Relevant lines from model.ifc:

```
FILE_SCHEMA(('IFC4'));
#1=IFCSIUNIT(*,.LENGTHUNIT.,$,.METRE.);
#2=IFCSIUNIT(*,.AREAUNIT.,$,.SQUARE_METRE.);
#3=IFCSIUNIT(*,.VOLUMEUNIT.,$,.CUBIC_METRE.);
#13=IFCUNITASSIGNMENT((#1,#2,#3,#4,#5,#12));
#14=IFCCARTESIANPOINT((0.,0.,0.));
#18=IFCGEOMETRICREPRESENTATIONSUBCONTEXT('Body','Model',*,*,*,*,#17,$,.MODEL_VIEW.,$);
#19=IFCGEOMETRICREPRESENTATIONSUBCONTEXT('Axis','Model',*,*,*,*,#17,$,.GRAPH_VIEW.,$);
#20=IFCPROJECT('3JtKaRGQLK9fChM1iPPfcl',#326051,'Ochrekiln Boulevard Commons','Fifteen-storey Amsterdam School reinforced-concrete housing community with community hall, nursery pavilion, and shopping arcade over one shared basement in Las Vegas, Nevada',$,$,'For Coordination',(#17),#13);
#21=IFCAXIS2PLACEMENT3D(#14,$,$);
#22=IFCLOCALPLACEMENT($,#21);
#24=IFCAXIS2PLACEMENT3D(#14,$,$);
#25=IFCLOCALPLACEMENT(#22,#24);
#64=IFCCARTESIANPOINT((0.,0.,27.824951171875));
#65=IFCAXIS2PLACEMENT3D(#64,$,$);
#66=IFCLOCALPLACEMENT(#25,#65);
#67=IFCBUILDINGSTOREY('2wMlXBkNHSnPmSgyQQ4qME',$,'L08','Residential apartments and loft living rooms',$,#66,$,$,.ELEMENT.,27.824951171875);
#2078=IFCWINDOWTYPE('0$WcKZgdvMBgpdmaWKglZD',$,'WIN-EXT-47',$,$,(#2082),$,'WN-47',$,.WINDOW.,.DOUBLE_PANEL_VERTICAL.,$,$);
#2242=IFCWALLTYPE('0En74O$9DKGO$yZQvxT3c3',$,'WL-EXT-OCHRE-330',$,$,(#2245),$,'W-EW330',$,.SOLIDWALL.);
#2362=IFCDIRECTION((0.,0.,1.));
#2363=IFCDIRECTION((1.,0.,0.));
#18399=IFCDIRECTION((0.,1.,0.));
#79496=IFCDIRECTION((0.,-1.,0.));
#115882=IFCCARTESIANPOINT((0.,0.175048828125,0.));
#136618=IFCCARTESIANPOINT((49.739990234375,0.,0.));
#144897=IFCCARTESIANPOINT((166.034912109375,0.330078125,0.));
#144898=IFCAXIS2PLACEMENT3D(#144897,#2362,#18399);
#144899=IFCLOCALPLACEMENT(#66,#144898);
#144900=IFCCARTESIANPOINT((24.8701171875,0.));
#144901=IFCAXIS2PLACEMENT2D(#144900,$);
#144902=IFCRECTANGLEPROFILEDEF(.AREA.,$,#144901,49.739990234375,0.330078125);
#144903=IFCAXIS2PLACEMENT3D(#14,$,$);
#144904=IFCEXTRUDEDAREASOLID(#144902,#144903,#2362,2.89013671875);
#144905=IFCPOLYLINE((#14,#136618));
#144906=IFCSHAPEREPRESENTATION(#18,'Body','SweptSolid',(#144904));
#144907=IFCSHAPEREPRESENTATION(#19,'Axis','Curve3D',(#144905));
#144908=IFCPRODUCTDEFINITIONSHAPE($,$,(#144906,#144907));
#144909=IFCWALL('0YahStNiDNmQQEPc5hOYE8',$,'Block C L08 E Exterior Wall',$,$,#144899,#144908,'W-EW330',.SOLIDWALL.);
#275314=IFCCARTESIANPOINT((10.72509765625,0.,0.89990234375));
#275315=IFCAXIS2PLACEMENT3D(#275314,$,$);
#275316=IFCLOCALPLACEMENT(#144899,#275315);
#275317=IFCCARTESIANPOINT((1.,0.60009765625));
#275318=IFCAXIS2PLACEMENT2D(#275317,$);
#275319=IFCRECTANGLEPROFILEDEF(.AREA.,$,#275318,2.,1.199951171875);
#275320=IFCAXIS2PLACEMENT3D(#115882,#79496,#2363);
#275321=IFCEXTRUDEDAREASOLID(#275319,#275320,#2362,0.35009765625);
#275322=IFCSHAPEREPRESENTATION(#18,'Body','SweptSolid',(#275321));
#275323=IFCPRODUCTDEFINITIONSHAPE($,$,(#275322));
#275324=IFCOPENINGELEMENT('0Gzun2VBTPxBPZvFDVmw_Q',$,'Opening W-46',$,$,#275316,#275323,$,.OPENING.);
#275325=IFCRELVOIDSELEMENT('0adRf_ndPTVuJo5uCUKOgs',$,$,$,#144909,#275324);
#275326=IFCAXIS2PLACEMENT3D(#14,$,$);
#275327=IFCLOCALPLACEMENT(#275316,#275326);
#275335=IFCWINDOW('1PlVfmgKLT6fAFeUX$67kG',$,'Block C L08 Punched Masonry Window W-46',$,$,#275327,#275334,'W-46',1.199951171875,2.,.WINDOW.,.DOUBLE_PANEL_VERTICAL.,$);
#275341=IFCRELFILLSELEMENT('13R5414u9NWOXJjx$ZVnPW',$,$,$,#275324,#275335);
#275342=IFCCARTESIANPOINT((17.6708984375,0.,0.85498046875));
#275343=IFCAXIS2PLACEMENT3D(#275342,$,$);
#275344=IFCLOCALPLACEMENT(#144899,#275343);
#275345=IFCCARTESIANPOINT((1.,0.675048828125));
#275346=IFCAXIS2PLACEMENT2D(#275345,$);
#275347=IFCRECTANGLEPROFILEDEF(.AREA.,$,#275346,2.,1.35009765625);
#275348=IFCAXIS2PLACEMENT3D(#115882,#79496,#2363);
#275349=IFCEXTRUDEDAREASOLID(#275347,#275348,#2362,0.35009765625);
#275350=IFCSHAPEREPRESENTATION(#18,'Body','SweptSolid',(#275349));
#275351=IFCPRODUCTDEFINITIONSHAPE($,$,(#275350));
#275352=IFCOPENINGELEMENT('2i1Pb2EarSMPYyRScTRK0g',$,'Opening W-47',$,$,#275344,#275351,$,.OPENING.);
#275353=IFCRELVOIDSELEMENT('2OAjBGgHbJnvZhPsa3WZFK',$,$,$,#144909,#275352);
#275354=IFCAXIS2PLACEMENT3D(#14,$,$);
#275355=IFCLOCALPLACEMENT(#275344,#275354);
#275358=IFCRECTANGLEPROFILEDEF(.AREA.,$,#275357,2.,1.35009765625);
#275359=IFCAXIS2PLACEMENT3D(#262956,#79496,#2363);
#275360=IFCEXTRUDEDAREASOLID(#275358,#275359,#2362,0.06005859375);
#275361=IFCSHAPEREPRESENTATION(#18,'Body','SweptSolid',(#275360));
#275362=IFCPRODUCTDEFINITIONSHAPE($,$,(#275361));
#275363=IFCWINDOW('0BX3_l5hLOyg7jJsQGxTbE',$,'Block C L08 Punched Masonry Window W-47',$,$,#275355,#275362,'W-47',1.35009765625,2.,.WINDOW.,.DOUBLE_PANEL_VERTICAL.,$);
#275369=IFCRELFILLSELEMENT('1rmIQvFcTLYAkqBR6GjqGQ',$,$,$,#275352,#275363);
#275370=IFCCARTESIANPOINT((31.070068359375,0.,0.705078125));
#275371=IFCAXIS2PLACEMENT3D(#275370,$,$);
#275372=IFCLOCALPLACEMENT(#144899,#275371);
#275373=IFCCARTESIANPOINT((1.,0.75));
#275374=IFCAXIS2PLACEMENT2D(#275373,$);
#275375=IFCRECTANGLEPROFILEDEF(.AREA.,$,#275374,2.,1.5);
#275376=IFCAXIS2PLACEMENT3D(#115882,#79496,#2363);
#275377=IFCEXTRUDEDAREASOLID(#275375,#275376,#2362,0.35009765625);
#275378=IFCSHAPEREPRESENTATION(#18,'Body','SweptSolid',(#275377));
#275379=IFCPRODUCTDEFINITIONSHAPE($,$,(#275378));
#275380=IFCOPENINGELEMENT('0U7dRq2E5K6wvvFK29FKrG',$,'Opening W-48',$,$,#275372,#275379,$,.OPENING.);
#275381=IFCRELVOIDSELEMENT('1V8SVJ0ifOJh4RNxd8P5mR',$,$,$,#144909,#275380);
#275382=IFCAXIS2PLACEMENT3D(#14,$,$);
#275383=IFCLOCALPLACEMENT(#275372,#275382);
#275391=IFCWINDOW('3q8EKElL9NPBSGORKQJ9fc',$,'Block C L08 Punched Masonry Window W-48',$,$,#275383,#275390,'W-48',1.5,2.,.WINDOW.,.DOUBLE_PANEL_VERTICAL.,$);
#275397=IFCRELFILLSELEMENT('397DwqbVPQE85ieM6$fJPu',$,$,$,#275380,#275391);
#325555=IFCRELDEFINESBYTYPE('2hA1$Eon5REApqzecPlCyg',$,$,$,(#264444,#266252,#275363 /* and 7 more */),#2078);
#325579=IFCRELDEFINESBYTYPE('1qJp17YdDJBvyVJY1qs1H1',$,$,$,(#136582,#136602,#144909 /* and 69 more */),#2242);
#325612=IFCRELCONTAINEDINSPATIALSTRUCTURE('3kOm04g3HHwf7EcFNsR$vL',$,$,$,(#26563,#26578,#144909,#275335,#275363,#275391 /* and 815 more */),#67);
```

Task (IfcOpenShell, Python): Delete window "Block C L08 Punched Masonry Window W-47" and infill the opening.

```python
import ifcopenshell
import ifcopenshell.api.feature
import ifcopenshell.api.root
import ifcopenshell.geom
import ifcopenshell.util.shape

model = ifcopenshell.open("model.ifc")
settings = ifcopenshell.geom.settings()


def volume(element):
    """Net volume in cubic metres, openings subtracted."""
    shape = ifcopenshell.geom.create_shape(settings, element)
    return ifcopenshell.util.shape.get_volume(shape.geometry)


window = model.by_guid("0BX3_l5hLOyg7jJsQGxTbE")
opening = window.FillsVoids[0].RelatingOpeningElement
wall = opening.VoidsElements[0].RelatingBuildingElement
before = volume(wall)

ifcopenshell.api.root.remove_product(model, product=window)
ifcopenshell.api.feature.remove_feature(model, feature=opening)

after = volume(wall)

print(f"wall volume {before:.3f} -> {after:.3f} m3")

model.write("model_edited.ifc")
```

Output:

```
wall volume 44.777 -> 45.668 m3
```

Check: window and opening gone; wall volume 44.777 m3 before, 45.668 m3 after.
